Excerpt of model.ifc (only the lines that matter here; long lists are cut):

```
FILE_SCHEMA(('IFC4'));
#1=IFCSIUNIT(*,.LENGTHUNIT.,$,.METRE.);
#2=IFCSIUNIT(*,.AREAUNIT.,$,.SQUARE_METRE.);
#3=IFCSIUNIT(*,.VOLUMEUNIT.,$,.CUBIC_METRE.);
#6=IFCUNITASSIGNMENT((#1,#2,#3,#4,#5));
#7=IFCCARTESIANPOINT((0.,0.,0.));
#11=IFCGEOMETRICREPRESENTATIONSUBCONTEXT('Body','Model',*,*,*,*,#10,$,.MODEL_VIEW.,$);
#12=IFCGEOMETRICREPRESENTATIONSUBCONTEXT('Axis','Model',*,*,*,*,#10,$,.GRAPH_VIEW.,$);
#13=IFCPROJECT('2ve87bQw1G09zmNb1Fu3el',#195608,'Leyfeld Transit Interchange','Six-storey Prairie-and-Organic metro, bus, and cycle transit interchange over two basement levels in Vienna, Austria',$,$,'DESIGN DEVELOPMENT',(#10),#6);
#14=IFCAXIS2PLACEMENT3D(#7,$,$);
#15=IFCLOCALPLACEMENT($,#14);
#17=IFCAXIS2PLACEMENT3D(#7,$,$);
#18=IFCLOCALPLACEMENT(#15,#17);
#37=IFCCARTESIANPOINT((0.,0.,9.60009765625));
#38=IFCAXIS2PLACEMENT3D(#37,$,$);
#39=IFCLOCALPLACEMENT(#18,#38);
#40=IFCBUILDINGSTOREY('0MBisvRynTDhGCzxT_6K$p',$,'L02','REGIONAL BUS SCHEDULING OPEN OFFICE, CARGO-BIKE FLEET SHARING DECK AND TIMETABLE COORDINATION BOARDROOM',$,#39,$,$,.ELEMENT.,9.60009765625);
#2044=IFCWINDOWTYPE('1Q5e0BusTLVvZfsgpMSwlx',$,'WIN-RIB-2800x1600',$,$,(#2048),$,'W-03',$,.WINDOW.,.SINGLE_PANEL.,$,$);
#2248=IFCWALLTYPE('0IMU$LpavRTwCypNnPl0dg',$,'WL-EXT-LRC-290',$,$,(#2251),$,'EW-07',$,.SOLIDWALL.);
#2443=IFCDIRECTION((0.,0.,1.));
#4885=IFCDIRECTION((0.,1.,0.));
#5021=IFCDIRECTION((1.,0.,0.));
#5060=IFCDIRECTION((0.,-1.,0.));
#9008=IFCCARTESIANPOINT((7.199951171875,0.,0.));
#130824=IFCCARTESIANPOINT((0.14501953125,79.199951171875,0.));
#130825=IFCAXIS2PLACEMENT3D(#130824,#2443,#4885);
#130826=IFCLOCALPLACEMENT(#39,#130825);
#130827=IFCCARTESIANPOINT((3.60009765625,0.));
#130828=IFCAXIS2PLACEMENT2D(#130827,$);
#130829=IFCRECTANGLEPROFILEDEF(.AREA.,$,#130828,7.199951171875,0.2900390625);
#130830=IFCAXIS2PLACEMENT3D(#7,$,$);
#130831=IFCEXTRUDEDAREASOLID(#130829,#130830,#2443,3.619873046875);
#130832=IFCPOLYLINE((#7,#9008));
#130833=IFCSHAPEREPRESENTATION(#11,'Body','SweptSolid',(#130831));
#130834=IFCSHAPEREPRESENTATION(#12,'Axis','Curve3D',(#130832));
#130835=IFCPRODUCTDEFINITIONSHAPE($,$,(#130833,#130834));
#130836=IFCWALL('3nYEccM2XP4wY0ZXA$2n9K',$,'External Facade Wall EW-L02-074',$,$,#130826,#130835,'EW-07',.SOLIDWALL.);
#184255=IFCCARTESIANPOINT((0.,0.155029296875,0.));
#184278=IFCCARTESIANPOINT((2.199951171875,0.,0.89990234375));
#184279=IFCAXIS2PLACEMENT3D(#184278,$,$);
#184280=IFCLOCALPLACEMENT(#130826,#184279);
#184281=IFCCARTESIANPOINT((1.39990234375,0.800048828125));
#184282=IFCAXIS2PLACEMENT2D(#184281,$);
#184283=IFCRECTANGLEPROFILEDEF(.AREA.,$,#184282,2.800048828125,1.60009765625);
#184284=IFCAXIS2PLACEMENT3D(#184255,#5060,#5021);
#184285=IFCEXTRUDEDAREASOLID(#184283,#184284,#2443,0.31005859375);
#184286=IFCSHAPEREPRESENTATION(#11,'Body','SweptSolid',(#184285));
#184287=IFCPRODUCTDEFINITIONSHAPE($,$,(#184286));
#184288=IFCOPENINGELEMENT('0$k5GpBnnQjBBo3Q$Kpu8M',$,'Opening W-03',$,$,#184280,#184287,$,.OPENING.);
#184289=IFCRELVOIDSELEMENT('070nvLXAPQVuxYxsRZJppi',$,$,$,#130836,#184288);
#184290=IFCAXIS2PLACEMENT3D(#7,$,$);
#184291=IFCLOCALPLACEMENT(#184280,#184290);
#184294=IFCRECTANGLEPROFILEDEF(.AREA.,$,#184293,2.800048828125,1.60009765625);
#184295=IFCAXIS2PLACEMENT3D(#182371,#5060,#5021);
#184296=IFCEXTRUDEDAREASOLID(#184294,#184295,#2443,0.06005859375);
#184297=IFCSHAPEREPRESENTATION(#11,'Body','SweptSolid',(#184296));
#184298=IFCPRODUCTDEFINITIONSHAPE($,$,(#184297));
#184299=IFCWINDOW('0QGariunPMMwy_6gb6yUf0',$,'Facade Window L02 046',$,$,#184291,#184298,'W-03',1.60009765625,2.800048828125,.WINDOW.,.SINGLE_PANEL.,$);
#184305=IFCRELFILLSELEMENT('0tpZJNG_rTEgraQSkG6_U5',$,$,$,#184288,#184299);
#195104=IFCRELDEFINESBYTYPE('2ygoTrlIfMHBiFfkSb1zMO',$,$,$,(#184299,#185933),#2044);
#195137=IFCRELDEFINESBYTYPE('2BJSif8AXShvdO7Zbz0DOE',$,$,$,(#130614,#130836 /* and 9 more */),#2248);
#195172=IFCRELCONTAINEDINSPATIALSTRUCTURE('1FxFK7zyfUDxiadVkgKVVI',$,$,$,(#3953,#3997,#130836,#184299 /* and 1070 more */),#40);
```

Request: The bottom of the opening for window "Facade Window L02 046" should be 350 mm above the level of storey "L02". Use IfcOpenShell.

```python
import numpy as np
import ifcopenshell
import ifcopenshell.api.geometry
import ifcopenshell.geom
import ifcopenshell.util.element
import ifcopenshell.util.placement
import ifcopenshell.util.shape
import ifcopenshell.util.unit

model = ifcopenshell.open("model.ifc")
unit_scale = ifcopenshell.util.unit.calculate_unit_scale(model)

window = model.by_guid("0QGariunPMMwy_6gb6yUf0")
opening = window.FillsVoids[0].RelatingOpeningElement
storey = ifcopenshell.util.element.get_container(window, ifc_class="IfcBuildingStorey")
level = ifcopenshell.util.placement.get_local_placement(storey.ObjectPlacement)[2, 3]

# The opening's origin need not be at the sill, so measure its lowest point.
shape = ifcopenshell.geom.create_shape(ifcopenshell.geom.settings(), opening)
bottom = ifcopenshell.util.shape.get_shape_bottom_elevation(shape, shape.geometry) / unit_scale
dz = level + 0.35 - bottom

shift = np.array([0.0, 0.0, dz])
# The window is placed relative to its opening, so it follows when the opening moves.
matrix = ifcopenshell.util.placement.get_local_placement(opening.ObjectPlacement)
matrix[:3, 3] += shift
ifcopenshell.api.geometry.edit_object_placement(
    model, product=opening, matrix=matrix, is_si=False, should_transform_children=True
)

print(f"moved by {dz * unit_scale:+.3f} m")

model.write("model_v2.ifc")
```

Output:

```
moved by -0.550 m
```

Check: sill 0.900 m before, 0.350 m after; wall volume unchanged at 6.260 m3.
